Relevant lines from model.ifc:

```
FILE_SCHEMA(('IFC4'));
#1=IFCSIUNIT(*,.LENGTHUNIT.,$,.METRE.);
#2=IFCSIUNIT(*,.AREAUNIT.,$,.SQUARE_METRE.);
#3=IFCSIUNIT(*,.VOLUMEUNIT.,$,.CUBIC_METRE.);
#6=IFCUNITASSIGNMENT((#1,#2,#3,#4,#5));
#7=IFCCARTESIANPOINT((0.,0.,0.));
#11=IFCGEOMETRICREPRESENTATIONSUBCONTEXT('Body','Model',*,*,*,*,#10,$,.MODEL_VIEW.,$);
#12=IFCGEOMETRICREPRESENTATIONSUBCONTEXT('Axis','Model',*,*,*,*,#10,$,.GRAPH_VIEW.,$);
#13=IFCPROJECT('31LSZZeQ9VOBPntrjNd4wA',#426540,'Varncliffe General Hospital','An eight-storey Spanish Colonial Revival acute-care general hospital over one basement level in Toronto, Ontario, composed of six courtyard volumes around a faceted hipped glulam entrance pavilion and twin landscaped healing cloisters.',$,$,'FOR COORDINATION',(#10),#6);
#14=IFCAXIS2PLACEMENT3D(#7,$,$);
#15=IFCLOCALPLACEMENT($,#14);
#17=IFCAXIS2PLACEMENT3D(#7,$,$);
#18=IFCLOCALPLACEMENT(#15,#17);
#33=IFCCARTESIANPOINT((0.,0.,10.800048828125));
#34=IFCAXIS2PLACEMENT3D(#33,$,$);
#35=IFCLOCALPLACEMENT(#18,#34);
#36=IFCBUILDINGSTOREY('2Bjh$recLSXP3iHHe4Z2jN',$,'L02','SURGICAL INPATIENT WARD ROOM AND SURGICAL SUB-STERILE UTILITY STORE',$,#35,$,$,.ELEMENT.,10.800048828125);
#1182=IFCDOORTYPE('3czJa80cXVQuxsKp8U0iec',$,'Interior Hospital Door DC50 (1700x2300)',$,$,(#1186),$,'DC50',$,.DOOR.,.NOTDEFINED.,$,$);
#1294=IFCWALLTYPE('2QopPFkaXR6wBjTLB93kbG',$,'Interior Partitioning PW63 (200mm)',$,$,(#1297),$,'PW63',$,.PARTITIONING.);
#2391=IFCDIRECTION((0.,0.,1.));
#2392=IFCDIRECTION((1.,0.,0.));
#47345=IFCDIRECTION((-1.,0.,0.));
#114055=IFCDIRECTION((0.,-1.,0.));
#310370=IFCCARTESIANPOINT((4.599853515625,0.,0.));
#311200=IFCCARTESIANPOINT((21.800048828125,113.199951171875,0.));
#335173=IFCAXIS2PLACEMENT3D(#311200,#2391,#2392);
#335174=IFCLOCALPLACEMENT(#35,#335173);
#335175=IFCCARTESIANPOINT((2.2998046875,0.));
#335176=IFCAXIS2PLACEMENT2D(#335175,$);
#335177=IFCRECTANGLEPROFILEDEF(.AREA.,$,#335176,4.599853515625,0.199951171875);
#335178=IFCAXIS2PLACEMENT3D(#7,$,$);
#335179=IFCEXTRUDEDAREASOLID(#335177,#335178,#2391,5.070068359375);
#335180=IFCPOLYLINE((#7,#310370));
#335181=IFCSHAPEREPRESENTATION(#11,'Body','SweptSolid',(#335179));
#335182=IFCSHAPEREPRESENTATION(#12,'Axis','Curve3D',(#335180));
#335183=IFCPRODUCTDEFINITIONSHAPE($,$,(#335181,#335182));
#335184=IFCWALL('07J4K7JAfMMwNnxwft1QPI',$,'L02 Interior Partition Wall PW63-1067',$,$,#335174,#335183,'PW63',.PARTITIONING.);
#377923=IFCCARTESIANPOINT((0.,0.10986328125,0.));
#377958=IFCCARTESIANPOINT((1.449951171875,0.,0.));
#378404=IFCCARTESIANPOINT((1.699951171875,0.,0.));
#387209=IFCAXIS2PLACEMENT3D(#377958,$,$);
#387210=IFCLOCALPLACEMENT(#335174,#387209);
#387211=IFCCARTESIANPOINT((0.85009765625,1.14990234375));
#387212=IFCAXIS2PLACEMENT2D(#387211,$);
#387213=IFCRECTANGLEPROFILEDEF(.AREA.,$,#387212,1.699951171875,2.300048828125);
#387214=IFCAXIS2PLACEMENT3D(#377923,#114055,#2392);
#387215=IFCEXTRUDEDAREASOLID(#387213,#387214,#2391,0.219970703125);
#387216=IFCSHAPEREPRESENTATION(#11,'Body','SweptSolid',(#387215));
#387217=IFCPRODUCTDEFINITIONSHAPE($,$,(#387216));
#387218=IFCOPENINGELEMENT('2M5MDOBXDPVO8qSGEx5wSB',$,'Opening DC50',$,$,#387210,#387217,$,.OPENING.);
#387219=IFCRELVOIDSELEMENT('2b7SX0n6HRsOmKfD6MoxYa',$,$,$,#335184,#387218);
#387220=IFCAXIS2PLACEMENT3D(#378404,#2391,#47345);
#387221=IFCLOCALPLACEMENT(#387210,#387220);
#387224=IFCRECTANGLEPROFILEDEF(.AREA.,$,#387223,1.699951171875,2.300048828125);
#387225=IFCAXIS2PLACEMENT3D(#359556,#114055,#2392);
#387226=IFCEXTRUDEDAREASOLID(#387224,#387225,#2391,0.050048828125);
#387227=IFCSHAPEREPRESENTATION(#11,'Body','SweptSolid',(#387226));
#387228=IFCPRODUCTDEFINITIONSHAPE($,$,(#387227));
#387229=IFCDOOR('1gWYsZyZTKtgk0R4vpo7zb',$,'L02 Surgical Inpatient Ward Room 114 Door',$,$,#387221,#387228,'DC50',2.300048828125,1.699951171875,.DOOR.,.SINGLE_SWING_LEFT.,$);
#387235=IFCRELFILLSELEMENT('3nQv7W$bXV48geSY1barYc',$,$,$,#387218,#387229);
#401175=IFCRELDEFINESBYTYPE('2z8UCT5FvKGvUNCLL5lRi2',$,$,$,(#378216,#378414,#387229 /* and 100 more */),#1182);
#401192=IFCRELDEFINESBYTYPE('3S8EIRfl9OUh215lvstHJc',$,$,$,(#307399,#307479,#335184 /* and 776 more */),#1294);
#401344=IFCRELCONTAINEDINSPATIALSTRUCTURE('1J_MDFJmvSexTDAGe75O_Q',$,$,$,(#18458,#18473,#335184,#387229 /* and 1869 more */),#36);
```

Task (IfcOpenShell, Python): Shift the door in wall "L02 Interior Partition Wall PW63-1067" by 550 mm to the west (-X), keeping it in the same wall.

```python
import ifcopenshell
import ifcopenshell.api.geometry
import ifcopenshell.util.placement

model = ifcopenshell.open("model.ifc")

door = model.by_guid("1gWYsZyZTKtgk0R4vpo7zb")
opening = door.FillsVoids[0].RelatingOpeningElement
wall = opening.VoidsElements[0].RelatingBuildingElement

wall_matrix = ifcopenshell.util.placement.get_local_placement(wall.ObjectPlacement)
shift = wall_matrix[:3, 0] * -0.55
before = ifcopenshell.util.placement.get_local_placement(door.ObjectPlacement)[:3, 3].copy()

# The door is placed relative to its opening, so it follows when the opening moves.
matrix = ifcopenshell.util.placement.get_local_placement(opening.ObjectPlacement)
matrix[:3, 3] += shift
ifcopenshell.api.geometry.edit_object_placement(
    model, product=opening, matrix=matrix, is_si=False, should_transform_children=True
)

after = ifcopenshell.util.placement.get_local_placement(door.ObjectPlacement)[:3, 3]
print("door moved by", (after - before).round(3) + 0.0)

model.write("model_v2.ifc")
```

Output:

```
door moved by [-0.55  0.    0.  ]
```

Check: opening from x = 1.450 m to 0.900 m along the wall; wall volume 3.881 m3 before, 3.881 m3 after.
